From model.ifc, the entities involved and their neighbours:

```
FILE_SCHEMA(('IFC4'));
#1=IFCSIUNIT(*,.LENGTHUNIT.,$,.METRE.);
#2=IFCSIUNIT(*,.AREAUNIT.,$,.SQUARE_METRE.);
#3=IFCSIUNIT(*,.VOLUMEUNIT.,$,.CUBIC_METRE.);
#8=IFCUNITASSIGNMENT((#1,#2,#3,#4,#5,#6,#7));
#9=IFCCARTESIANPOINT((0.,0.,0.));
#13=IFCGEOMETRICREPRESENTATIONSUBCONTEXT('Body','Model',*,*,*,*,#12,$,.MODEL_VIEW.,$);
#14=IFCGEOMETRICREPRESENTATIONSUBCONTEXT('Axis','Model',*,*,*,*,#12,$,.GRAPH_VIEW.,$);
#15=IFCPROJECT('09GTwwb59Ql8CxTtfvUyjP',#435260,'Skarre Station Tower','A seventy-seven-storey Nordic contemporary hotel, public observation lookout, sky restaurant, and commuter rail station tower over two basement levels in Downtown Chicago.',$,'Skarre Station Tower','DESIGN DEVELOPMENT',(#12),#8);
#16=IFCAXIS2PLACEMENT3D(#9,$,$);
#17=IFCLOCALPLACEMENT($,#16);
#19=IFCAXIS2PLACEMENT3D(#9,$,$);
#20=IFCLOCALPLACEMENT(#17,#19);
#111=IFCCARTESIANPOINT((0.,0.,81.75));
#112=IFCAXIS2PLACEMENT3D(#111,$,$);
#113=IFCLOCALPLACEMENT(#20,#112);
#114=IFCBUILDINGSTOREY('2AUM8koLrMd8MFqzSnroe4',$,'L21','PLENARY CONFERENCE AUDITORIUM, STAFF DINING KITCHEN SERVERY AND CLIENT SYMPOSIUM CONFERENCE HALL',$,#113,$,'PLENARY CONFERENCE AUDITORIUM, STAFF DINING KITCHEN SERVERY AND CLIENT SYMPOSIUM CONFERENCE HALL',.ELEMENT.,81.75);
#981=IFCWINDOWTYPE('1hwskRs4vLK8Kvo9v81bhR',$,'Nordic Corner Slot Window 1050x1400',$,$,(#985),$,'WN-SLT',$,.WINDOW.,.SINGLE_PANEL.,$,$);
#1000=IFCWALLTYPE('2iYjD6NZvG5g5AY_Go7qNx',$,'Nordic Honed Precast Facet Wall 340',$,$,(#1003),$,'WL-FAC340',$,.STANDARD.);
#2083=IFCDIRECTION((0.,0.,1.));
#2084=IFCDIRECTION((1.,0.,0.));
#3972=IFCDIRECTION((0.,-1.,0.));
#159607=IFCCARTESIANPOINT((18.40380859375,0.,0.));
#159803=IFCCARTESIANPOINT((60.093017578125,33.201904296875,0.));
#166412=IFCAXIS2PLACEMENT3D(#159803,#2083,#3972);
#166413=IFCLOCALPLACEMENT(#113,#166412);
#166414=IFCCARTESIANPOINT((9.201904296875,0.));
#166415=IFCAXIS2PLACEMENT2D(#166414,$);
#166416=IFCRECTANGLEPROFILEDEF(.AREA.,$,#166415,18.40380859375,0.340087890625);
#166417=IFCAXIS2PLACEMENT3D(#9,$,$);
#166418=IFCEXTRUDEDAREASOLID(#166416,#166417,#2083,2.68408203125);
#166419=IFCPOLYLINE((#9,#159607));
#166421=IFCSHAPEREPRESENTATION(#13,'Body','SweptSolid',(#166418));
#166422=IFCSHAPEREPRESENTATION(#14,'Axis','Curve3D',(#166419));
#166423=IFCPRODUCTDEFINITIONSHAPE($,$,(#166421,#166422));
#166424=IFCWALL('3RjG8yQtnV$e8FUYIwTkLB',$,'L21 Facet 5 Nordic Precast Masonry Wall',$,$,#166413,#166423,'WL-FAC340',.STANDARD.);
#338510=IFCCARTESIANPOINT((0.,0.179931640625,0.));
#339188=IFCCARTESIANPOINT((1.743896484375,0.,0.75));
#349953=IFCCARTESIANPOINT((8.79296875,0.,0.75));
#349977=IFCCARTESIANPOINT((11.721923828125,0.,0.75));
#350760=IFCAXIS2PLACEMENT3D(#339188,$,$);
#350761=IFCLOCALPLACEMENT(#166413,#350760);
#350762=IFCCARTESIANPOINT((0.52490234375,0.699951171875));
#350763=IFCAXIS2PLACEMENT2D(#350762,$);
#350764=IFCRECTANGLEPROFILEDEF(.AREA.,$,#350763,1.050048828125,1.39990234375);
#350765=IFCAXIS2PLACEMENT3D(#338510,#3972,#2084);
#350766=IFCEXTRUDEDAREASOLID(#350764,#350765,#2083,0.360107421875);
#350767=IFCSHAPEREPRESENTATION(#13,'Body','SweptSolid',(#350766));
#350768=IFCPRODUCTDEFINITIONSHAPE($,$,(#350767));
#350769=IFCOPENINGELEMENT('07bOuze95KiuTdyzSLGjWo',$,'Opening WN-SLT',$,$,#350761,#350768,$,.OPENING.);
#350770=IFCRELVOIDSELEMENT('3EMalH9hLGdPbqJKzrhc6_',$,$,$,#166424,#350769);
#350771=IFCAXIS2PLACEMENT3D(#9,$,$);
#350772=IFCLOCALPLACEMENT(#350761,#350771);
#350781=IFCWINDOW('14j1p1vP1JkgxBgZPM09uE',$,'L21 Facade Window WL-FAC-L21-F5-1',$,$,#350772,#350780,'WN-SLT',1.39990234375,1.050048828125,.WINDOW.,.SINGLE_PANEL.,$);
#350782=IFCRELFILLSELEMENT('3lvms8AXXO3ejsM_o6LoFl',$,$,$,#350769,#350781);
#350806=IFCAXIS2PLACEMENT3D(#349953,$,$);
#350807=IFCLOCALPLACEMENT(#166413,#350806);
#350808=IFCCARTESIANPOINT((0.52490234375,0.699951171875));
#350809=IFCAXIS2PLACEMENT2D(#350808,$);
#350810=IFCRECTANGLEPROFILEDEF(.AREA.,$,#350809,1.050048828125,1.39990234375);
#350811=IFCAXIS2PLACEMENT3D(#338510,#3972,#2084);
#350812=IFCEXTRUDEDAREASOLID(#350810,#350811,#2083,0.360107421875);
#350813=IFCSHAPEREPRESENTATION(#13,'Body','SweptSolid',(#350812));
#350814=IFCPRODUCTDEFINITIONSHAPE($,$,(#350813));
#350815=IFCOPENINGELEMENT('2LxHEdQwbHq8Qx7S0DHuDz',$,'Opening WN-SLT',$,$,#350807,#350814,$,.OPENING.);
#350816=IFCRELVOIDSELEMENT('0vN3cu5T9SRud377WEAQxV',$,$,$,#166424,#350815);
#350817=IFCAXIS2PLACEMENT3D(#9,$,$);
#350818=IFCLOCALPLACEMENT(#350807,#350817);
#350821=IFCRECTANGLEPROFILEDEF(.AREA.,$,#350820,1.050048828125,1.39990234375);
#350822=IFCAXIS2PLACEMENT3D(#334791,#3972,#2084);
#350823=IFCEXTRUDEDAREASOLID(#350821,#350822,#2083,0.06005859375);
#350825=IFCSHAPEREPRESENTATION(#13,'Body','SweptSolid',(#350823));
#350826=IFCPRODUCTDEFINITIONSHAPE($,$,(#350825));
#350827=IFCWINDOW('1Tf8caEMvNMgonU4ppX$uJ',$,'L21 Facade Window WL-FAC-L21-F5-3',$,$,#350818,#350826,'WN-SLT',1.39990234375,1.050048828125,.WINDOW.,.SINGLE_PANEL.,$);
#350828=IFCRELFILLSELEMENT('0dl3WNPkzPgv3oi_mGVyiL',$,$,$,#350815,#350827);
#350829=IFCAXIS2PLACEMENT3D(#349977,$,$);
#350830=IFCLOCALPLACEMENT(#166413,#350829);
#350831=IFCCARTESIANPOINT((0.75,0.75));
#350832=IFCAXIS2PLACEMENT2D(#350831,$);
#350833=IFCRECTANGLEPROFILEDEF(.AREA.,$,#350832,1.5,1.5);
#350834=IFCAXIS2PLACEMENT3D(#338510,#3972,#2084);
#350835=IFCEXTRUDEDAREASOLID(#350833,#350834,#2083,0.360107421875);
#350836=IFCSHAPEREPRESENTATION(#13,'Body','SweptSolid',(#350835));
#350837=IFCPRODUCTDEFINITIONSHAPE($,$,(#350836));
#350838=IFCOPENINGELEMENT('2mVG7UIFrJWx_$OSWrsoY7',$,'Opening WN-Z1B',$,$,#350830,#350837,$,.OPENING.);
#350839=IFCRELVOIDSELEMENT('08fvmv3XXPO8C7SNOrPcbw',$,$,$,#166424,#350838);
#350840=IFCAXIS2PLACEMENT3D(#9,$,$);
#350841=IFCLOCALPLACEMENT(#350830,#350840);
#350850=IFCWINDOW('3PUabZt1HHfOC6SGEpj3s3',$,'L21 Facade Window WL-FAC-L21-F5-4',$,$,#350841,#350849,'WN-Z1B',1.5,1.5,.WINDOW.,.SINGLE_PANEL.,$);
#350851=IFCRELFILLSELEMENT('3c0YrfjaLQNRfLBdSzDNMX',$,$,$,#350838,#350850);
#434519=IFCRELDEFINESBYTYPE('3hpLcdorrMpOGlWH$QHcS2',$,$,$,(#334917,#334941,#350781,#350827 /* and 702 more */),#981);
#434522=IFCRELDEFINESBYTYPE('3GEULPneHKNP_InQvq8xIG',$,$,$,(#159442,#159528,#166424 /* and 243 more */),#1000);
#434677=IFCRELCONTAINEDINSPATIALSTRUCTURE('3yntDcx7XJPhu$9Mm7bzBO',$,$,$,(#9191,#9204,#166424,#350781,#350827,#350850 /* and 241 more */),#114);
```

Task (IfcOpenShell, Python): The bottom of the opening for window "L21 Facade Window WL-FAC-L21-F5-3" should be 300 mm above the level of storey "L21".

```python
import numpy as np
import ifcopenshell
import ifcopenshell.api.geometry
import ifcopenshell.geom
import ifcopenshell.util.element
import ifcopenshell.util.placement
import ifcopenshell.util.shape
import ifcopenshell.util.unit

model = ifcopenshell.open("model.ifc")
unit_scale = ifcopenshell.util.unit.calculate_unit_scale(model)

window = model.by_id(350827)
opening = window.FillsVoids[0].RelatingOpeningElement
storey = ifcopenshell.util.element.get_container(window, ifc_class="IfcBuildingStorey")
level = ifcopenshell.util.placement.get_local_placement(storey.ObjectPlacement)[2, 3]

# The opening's origin need not be at the sill, so measure its lowest point.
shape = ifcopenshell.geom.create_shape(ifcopenshell.geom.settings(), opening)
bottom = ifcopenshell.util.shape.get_shape_bottom_elevation(shape, shape.geometry) / unit_scale
dz = level + 0.3 - bottom

shift = np.array([0.0, 0.0, dz])
# The window is placed relative to its opening, so it follows when the opening moves.
matrix = ifcopenshell.util.placement.get_local_placement(opening.ObjectPlacement)
matrix[:3, 3] += shift
ifcopenshell.api.geometry.edit_object_placement(
    model, product=opening, matrix=matrix, is_si=False, should_transform_children=True
)

print(f"moved by {dz * unit_scale:+.3f} m")

model.write("model_rev.ifc")
```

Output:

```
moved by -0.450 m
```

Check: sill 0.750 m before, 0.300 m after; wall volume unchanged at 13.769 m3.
